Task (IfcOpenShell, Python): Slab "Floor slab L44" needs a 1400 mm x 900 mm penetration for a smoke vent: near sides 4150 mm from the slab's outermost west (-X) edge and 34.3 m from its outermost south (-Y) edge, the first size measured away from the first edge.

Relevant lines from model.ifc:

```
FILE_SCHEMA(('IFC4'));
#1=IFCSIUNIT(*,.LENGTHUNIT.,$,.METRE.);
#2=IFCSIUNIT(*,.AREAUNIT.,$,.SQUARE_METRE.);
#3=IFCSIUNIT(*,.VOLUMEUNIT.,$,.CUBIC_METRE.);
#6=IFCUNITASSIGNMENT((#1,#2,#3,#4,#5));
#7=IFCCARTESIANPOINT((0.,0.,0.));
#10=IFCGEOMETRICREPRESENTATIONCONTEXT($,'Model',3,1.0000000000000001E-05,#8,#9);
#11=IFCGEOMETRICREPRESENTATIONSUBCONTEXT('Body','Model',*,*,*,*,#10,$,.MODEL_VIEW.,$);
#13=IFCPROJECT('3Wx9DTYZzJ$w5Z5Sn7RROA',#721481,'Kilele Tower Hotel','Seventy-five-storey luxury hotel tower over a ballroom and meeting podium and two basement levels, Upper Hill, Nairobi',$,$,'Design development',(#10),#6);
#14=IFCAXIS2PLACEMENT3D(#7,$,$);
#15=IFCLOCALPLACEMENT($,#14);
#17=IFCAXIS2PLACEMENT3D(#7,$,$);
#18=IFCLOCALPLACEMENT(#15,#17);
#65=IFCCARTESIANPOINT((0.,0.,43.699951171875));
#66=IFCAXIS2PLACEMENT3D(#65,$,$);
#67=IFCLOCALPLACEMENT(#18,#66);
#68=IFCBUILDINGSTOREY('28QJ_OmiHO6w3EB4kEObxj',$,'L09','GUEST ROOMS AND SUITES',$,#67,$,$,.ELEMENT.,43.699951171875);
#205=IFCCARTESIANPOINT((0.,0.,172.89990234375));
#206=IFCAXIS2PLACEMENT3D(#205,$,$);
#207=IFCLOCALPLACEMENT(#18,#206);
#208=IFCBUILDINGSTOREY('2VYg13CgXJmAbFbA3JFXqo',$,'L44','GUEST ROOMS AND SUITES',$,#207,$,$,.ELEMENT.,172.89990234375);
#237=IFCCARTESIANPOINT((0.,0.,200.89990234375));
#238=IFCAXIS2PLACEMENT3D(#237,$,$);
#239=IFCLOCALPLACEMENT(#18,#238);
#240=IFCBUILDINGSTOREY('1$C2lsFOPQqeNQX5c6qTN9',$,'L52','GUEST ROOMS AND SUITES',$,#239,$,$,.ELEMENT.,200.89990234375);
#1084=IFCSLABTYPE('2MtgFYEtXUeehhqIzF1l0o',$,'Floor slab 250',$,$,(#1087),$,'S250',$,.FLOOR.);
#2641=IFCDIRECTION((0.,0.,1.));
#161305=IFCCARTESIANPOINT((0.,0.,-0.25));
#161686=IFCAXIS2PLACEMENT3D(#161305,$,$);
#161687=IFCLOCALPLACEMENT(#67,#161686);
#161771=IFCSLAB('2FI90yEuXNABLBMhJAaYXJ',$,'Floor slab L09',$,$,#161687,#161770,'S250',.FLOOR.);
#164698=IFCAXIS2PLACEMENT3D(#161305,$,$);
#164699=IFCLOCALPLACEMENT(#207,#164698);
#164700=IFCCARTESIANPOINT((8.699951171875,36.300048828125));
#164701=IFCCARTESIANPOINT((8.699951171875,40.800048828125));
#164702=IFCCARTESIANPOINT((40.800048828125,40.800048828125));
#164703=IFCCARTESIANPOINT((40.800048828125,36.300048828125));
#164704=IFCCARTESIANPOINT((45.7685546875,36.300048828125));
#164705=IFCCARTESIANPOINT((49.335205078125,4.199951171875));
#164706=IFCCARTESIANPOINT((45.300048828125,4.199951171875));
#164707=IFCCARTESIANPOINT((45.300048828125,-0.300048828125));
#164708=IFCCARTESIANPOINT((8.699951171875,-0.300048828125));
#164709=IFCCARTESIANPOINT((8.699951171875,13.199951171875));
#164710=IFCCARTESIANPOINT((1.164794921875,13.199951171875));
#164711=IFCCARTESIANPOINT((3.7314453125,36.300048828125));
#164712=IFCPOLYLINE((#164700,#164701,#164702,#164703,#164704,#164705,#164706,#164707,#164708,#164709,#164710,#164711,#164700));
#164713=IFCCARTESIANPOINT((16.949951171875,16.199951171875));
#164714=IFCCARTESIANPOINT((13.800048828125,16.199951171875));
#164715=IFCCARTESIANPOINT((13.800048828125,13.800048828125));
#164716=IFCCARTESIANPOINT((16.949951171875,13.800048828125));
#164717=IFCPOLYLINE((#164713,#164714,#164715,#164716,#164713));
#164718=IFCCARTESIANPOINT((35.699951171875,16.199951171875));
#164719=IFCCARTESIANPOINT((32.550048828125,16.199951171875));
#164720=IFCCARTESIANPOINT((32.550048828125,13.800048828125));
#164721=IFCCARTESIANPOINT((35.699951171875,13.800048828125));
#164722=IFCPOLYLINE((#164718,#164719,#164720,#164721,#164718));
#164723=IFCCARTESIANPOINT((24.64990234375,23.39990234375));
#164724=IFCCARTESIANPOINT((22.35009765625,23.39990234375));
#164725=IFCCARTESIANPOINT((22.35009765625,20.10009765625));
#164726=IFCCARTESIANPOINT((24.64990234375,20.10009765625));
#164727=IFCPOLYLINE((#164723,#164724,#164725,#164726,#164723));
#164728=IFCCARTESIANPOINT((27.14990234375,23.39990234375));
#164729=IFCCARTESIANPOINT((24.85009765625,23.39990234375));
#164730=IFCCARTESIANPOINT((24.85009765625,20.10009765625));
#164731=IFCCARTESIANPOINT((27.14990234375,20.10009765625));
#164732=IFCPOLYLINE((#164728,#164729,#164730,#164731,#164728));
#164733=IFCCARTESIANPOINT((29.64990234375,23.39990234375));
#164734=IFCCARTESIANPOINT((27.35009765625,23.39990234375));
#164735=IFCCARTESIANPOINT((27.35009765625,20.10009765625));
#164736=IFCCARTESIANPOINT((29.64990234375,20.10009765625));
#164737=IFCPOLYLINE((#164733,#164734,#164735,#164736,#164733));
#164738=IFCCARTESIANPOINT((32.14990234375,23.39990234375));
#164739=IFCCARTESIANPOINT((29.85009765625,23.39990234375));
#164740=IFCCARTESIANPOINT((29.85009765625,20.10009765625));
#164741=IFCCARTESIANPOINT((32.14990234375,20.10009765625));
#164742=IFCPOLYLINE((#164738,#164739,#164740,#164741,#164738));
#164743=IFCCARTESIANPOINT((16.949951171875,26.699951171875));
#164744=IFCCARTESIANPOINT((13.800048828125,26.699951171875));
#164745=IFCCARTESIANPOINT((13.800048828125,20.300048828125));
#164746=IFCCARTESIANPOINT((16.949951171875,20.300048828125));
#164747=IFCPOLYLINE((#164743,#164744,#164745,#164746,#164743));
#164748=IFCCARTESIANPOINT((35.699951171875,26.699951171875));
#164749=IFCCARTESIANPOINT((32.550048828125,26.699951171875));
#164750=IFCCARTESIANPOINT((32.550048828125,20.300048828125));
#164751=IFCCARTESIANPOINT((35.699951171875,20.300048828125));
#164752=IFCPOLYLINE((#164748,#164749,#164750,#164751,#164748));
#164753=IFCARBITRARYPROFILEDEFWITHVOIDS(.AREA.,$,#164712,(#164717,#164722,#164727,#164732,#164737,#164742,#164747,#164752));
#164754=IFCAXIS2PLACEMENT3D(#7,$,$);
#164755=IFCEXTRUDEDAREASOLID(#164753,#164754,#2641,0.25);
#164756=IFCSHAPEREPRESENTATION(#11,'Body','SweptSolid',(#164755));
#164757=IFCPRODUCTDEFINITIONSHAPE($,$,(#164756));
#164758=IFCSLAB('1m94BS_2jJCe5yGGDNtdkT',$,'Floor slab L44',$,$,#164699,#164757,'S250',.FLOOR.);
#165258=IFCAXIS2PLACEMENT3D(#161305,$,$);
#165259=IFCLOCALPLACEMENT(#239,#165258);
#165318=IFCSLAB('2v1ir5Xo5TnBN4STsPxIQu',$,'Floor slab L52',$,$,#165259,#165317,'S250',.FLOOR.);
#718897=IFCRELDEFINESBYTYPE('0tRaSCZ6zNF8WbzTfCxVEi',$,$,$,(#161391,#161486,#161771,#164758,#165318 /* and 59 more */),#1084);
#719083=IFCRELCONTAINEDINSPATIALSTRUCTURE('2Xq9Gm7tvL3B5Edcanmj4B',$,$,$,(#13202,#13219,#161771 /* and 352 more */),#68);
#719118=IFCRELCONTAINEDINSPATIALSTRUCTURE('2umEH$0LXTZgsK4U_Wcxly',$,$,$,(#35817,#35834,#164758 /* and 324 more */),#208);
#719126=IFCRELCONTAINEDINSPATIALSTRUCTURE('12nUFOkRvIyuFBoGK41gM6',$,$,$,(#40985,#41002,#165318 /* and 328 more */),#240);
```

```python
import numpy as np
import ifcopenshell
import ifcopenshell.api.feature
import ifcopenshell.api.geometry
import ifcopenshell.api.root
import ifcopenshell.geom
import ifcopenshell.util.placement
import ifcopenshell.util.representation
import ifcopenshell.util.shape
import ifcopenshell.util.unit

model = ifcopenshell.open("model.ifc")
unit_scale = ifcopenshell.util.unit.calculate_unit_scale(model)
settings = ifcopenshell.geom.settings()


def volume(element):
    """Net volume in cubic metres, openings subtracted."""
    shape = ifcopenshell.geom.create_shape(settings, element)
    return ifcopenshell.util.shape.get_volume(shape.geometry)


slab = model.by_guid("1m94BS_2jJCe5yGGDNtdkT")
before = volume(slab)

# Extent in the slab's own axes, in metres. The edges named are its -X and -Y sides.
slab_shape = ifcopenshell.geom.create_shape(settings, slab)
vertices = ifcopenshell.util.shape.get_vertices(slab_shape.geometry)
x_min, y_min, bottom = vertices.min(axis=0)
top = vertices[:, 2].max()

opening = ifcopenshell.api.root.create_entity(model, ifc_class="IfcOpeningElement", name="Smoke vent opening", predefined_type="OPENING")
context = ifcopenshell.util.representation.get_context(model, "Model", "Body", "MODEL_VIEW")
width, depth = 1.4, 0.9
outline = [(0.0, 0.0), (width, 0.0), (width, depth), (0.0, depth), (0.0, 0.0)]
# Overshoot both faces by 50 mm so the cut is clean.
shape = ifcopenshell.api.geometry.add_slab_representation(
    model, context=context, depth=top - bottom + 0.1, polyline=outline
)
ifcopenshell.api.geometry.assign_representation(model, product=opening, representation=shape)

matrix = ifcopenshell.util.placement.get_local_placement(slab.ObjectPlacement)
matrix[:, 3] = matrix @ np.append(np.array([x_min + 4.15, y_min + 34.3, bottom - 0.05]) / unit_scale, 1.0)
ifcopenshell.api.geometry.edit_object_placement(model, product=opening, matrix=matrix, is_si=False)
ifcopenshell.api.feature.add_feature(model, feature=opening, element=slab)

after = volume(slab)

print(f"slab volume {before:.3f} -> {after:.3f} m3")

model.write("model_updated.ifc")
```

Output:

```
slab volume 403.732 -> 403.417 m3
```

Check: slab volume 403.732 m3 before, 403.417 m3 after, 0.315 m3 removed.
